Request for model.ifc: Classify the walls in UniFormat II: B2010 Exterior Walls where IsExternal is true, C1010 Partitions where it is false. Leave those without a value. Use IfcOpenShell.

First a look at what the model holds.

```python
import ifcopenshell
import ifcopenshell.util.element

model = ifcopenshell.open("model.ifc")
print(model.schema)
print("classifications:", [c.Name for c in model.by_type("IfcClassification")])
values = [ifcopenshell.util.element.get_pset(e, "Pset_WallCommon", "IsExternal") for e in model.by_type("IfcWall")]
for value in (True, False, None):
    print("IsExternal", value, values.count(value))
```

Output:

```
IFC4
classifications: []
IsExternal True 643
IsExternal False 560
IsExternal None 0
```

```python
import ifcopenshell
import ifcopenshell.api.classification
import ifcopenshell.util.element

model = ifcopenshell.open("model.ifc")

system = ifcopenshell.api.classification.add_classification(model, classification="UniFormat II")

walls = model.by_type("IfcWall")
external = {e: ifcopenshell.util.element.get_pset(e, "Pset_WallCommon", "IsExternal") for e in walls}
for flag, code, name in ((True, "B2010", "Exterior Walls"), (False, "C1010", "Partitions")):
    products = [e for e in walls if external[e] is flag]
    ifcopenshell.api.classification.add_reference(
        model, products=products, classification=system, identification=code, name=name
    )
    print(code, len(products))

model.write("model_edited.ifc")
```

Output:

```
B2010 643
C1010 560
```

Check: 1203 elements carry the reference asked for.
